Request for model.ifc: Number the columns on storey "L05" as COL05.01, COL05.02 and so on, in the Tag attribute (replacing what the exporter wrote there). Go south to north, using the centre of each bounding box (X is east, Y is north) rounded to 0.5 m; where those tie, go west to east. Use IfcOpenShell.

First a look at what the model holds.

```python
import ifcopenshell
import ifcopenshell.util.element
import ifcopenshell.util.placement

model = ifcopenshell.open("model.ifc")
print(model.schema)
storey = next(s for s in model.by_type("IfcBuildingStorey") if s.Name == "L05")
columns = [e for e in ifcopenshell.util.element.get_decomposition(storey) if e.is_a("IfcColumn")]
for e in sorted(columns, key=lambda e: e.id()):
    origin = ifcopenshell.util.placement.get_local_placement(e.ObjectPlacement)[:3, 3]
    print(e.id(), e.Tag, e.Name, origin.round(2) + 0.0, sep=" | ")
```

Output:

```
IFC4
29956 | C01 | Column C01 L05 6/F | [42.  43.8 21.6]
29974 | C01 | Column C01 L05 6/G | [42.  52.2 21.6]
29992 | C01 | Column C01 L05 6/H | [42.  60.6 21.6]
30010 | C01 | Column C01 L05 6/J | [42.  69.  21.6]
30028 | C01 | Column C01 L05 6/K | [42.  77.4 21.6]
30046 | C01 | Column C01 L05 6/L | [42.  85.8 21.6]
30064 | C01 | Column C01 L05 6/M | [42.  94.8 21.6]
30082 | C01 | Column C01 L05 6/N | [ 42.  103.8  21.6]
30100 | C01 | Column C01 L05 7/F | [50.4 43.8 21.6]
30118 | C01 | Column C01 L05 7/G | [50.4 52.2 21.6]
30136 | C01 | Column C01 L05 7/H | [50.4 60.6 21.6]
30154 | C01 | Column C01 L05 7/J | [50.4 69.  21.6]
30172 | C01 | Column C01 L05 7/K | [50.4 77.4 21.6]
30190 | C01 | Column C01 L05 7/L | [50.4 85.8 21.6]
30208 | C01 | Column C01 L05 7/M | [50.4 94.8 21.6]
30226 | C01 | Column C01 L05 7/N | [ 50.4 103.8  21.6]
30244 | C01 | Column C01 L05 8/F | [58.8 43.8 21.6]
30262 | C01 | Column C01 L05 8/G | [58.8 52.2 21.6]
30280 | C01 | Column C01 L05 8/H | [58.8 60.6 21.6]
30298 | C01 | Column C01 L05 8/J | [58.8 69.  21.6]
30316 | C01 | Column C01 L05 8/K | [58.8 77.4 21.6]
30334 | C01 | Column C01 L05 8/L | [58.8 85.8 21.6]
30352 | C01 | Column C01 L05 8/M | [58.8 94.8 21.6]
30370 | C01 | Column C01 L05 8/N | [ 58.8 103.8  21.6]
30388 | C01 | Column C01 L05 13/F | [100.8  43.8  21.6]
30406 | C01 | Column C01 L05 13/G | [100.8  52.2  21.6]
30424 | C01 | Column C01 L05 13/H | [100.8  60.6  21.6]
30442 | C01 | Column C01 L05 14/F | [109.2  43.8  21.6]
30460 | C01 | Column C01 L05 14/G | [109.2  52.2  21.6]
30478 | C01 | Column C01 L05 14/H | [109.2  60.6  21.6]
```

```python
import ifcopenshell
import ifcopenshell.geom
import ifcopenshell.util.element
import ifcopenshell.util.shape

model = ifcopenshell.open("model.ifc")
settings = ifcopenshell.geom.settings()
settings.set("use-world-coords", True)


def centre(element):
    shape = ifcopenshell.geom.create_shape(settings, element)
    return ifcopenshell.util.shape.get_bbox_centroid(shape.geometry)


storey = next(s for s in model.by_type("IfcBuildingStorey") if s.Name == "L05")
columns = [e for e in ifcopenshell.util.element.get_decomposition(storey) if e.is_a("IfcColumn")]

# Insertion points can sit at a corner or the storey origin, so sort by the geometry (in metres).
centres = {e: centre(e) for e in columns}
columns.sort(key=lambda e: (round(centres[e][1] / 0.5), centres[e][0]))

for i, e in enumerate(columns, start=1):
    number = f"COL05.{i:02d}"
    e.Tag = number
    print(e.id(), number)

model.write("model_edited.ifc")
```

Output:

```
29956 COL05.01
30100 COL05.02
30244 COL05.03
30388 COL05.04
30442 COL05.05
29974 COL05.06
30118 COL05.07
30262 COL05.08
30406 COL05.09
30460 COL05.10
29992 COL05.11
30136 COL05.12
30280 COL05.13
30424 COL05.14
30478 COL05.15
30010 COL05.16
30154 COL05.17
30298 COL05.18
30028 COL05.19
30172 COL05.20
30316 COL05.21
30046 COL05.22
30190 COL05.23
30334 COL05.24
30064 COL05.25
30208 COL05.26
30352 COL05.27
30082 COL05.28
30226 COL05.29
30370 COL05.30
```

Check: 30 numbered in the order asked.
